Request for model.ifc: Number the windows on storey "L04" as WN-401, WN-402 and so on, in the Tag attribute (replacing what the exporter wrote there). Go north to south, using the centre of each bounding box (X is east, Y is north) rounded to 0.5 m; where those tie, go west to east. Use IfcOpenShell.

First a look at what the model holds.

```python
import ifcopenshell
import ifcopenshell.util.element
import ifcopenshell.util.placement

model = ifcopenshell.open("model.ifc")
print(model.schema)
storey = next(s for s in model.by_type("IfcBuildingStorey") if s.Name == "L04")
windows = [e for e in ifcopenshell.util.element.get_decomposition(storey) if e.is_a("IfcWindow")]
for e in sorted(windows, key=lambda e: e.id()):
    origin = ifcopenshell.util.placement.get_local_placement(e.ObjectPlacement)[:3, 3]
    print(e.id(), e.Tag, e.Name, origin.round(2) + 0.0, sep=" | ")
```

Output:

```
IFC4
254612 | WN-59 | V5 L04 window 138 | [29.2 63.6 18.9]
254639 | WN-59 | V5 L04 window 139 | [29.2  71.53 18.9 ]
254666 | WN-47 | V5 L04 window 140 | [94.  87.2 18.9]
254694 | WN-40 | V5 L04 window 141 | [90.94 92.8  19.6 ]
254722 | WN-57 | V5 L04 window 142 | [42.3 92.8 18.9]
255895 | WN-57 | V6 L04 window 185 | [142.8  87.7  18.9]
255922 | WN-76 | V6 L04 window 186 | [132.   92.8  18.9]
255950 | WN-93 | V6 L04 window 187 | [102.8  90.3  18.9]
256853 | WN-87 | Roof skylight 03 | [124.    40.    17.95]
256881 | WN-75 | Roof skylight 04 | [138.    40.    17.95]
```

```python
import ifcopenshell
import ifcopenshell.geom
import ifcopenshell.util.element
import ifcopenshell.util.shape

model = ifcopenshell.open("model.ifc")
settings = ifcopenshell.geom.settings()
settings.set("use-world-coords", True)


def centre(element):
    shape = ifcopenshell.geom.create_shape(settings, element)
    return ifcopenshell.util.shape.get_bbox_centroid(shape.geometry)


storey = next(s for s in model.by_type("IfcBuildingStorey") if s.Name == "L04")
windows = [e for e in ifcopenshell.util.element.get_decomposition(storey) if e.is_a("IfcWindow")]

# Insertion points can sit at a corner or the storey origin, so sort by the geometry (in metres).
centres = {e: centre(e) for e in windows}
windows.sort(key=lambda e: (-round(centres[e][1] / 0.5), centres[e][0]))

for i, e in enumerate(windows, start=1):
    number = f"WN-4{i:02d}"
    e.Tag = number
    print(e.id(), number)

model.write("model-out.ifc")
```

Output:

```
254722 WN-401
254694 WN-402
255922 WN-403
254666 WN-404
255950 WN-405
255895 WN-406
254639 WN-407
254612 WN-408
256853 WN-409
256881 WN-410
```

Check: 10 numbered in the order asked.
